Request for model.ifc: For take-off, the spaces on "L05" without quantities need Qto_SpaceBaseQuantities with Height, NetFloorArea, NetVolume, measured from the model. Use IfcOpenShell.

First a look at what the model holds.

```python
import ifcopenshell
import ifcopenshell.util.element
import ifcopenshell.util.unit

model = ifcopenshell.open("model.ifc")
print(model.schema)
for unit_type in ("LENGTHUNIT", "AREAUNIT", "VOLUMEUNIT"):
    print(unit_type, ifcopenshell.util.unit.calculate_unit_scale(model, unit_type))
storey = next(s for s in model.by_type("IfcBuildingStorey") if s.Name == "L05")
spaces = [e for e in ifcopenshell.util.element.get_decomposition(storey) if e.is_a("IfcSpace")]
for e in sorted(spaces, key=lambda e: e.id()):
    print(e.id(), e.is_a(), e.Name, list(ifcopenshell.util.element.get_psets(e, qtos_only=True)), sep=" | ")
```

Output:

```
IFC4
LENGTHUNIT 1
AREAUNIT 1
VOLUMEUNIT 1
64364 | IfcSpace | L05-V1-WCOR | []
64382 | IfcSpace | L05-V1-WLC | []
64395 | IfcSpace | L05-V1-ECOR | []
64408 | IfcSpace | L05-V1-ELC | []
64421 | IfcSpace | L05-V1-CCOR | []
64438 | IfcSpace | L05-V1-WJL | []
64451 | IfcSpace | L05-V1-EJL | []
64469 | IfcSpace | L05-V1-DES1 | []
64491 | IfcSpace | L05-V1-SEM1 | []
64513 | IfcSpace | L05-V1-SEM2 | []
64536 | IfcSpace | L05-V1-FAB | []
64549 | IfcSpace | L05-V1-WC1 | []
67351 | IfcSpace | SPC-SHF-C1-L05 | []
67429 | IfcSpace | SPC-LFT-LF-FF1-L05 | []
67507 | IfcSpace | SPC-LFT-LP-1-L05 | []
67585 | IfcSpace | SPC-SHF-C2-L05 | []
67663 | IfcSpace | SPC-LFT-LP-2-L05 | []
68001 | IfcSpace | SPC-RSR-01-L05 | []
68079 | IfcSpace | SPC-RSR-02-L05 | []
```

```python
import ifcopenshell
import ifcopenshell.api.pset
import ifcopenshell.geom
import ifcopenshell.util.element
import ifcopenshell.util.shape
import ifcopenshell.util.unit

model = ifcopenshell.open("model.ifc")
unit_scale = ifcopenshell.util.unit.calculate_unit_scale(model)
area_scale = ifcopenshell.util.unit.calculate_unit_scale(model, "AREAUNIT")
volume_scale = ifcopenshell.util.unit.calculate_unit_scale(model, "VOLUMEUNIT")
settings = ifcopenshell.geom.settings()

storey = next(s for s in model.by_type("IfcBuildingStorey") if s.Name == "L05")
spaces = [e for e in ifcopenshell.util.element.get_decomposition(storey) if e.is_a("IfcSpace")]

for e in sorted(spaces, key=lambda e: e.id()):
    if ifcopenshell.util.element.get_psets(e, qtos_only=True, should_inherit=False):
        continue
    # Geometry comes back in metres, in the element's own axes.
    shape = ifcopenshell.geom.create_shape(settings, e)
    values = {
        "Height": ifcopenshell.util.shape.get_z(shape.geometry) / unit_scale,
        "NetFloorArea": ifcopenshell.util.shape.get_footprint_area(shape.geometry) / area_scale,
        "NetVolume": ifcopenshell.util.shape.get_volume(shape.geometry) / volume_scale,
    }
    qto = ifcopenshell.api.pset.add_qto(model, product=e, name="Qto_SpaceBaseQuantities")
    ifcopenshell.api.pset.edit_qto(model, qto=qto, properties=values)
    print(e.id(), {k: round(v, 3) for k, v in values.items()})

model.write("model_edited.ifc")
```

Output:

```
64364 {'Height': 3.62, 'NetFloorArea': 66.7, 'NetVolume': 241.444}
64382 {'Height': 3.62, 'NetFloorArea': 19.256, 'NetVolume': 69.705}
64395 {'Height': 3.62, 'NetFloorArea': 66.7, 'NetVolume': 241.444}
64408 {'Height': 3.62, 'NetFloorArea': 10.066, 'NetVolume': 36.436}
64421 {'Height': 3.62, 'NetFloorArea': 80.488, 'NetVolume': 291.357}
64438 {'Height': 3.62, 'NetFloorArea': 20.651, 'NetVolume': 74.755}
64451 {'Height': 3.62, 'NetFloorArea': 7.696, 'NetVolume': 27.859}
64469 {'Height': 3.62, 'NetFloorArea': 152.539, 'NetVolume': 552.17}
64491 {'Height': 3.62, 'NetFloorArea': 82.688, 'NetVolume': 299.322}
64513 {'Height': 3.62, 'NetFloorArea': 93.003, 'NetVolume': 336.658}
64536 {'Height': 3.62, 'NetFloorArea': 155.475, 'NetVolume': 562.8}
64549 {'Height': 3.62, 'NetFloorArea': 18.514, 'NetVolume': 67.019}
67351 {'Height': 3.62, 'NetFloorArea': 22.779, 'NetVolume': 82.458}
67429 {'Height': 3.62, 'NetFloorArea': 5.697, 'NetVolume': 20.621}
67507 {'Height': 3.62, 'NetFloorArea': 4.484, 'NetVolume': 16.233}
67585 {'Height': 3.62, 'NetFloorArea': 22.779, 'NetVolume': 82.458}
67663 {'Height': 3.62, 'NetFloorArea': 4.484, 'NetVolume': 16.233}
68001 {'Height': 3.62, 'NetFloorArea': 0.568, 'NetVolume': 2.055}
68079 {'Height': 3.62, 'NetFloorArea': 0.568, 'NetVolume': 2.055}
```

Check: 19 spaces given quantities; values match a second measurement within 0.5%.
